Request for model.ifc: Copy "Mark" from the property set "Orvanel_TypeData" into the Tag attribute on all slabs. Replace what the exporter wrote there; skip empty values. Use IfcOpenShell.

First a look at what the model holds.

```python
import ifcopenshell
import ifcopenshell.util.element

model = ifcopenshell.open("model.ifc")
print(model.schema)
slabs = model.by_type("IfcSlab")
print(len(slabs), "slabs")
for e in slabs[:8]:
    source = ifcopenshell.util.element.get_pset(e, "Orvanel_TypeData", "Mark")
    target = e.Tag
    print(e.id(), repr(source), repr(target), sep=" | ")
```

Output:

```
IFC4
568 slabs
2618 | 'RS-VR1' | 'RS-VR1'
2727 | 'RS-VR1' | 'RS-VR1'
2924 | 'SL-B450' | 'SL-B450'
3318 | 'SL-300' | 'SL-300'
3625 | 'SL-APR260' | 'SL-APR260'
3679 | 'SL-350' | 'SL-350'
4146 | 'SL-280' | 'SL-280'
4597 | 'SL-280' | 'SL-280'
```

```python
import ifcopenshell
import ifcopenshell.util.element

model = ifcopenshell.open("model.ifc")

count = 0
for e in model.by_type("IfcSlab"):
    value = ifcopenshell.util.element.get_pset(e, "Orvanel_TypeData", "Mark")
    current = e.Tag
    if not value or not value.strip() or current == value:
        continue
    e.Tag = value
    count += 1

print(count, "slabs updated")

model.write("model_v2.ifc")
```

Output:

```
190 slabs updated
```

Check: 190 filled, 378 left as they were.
